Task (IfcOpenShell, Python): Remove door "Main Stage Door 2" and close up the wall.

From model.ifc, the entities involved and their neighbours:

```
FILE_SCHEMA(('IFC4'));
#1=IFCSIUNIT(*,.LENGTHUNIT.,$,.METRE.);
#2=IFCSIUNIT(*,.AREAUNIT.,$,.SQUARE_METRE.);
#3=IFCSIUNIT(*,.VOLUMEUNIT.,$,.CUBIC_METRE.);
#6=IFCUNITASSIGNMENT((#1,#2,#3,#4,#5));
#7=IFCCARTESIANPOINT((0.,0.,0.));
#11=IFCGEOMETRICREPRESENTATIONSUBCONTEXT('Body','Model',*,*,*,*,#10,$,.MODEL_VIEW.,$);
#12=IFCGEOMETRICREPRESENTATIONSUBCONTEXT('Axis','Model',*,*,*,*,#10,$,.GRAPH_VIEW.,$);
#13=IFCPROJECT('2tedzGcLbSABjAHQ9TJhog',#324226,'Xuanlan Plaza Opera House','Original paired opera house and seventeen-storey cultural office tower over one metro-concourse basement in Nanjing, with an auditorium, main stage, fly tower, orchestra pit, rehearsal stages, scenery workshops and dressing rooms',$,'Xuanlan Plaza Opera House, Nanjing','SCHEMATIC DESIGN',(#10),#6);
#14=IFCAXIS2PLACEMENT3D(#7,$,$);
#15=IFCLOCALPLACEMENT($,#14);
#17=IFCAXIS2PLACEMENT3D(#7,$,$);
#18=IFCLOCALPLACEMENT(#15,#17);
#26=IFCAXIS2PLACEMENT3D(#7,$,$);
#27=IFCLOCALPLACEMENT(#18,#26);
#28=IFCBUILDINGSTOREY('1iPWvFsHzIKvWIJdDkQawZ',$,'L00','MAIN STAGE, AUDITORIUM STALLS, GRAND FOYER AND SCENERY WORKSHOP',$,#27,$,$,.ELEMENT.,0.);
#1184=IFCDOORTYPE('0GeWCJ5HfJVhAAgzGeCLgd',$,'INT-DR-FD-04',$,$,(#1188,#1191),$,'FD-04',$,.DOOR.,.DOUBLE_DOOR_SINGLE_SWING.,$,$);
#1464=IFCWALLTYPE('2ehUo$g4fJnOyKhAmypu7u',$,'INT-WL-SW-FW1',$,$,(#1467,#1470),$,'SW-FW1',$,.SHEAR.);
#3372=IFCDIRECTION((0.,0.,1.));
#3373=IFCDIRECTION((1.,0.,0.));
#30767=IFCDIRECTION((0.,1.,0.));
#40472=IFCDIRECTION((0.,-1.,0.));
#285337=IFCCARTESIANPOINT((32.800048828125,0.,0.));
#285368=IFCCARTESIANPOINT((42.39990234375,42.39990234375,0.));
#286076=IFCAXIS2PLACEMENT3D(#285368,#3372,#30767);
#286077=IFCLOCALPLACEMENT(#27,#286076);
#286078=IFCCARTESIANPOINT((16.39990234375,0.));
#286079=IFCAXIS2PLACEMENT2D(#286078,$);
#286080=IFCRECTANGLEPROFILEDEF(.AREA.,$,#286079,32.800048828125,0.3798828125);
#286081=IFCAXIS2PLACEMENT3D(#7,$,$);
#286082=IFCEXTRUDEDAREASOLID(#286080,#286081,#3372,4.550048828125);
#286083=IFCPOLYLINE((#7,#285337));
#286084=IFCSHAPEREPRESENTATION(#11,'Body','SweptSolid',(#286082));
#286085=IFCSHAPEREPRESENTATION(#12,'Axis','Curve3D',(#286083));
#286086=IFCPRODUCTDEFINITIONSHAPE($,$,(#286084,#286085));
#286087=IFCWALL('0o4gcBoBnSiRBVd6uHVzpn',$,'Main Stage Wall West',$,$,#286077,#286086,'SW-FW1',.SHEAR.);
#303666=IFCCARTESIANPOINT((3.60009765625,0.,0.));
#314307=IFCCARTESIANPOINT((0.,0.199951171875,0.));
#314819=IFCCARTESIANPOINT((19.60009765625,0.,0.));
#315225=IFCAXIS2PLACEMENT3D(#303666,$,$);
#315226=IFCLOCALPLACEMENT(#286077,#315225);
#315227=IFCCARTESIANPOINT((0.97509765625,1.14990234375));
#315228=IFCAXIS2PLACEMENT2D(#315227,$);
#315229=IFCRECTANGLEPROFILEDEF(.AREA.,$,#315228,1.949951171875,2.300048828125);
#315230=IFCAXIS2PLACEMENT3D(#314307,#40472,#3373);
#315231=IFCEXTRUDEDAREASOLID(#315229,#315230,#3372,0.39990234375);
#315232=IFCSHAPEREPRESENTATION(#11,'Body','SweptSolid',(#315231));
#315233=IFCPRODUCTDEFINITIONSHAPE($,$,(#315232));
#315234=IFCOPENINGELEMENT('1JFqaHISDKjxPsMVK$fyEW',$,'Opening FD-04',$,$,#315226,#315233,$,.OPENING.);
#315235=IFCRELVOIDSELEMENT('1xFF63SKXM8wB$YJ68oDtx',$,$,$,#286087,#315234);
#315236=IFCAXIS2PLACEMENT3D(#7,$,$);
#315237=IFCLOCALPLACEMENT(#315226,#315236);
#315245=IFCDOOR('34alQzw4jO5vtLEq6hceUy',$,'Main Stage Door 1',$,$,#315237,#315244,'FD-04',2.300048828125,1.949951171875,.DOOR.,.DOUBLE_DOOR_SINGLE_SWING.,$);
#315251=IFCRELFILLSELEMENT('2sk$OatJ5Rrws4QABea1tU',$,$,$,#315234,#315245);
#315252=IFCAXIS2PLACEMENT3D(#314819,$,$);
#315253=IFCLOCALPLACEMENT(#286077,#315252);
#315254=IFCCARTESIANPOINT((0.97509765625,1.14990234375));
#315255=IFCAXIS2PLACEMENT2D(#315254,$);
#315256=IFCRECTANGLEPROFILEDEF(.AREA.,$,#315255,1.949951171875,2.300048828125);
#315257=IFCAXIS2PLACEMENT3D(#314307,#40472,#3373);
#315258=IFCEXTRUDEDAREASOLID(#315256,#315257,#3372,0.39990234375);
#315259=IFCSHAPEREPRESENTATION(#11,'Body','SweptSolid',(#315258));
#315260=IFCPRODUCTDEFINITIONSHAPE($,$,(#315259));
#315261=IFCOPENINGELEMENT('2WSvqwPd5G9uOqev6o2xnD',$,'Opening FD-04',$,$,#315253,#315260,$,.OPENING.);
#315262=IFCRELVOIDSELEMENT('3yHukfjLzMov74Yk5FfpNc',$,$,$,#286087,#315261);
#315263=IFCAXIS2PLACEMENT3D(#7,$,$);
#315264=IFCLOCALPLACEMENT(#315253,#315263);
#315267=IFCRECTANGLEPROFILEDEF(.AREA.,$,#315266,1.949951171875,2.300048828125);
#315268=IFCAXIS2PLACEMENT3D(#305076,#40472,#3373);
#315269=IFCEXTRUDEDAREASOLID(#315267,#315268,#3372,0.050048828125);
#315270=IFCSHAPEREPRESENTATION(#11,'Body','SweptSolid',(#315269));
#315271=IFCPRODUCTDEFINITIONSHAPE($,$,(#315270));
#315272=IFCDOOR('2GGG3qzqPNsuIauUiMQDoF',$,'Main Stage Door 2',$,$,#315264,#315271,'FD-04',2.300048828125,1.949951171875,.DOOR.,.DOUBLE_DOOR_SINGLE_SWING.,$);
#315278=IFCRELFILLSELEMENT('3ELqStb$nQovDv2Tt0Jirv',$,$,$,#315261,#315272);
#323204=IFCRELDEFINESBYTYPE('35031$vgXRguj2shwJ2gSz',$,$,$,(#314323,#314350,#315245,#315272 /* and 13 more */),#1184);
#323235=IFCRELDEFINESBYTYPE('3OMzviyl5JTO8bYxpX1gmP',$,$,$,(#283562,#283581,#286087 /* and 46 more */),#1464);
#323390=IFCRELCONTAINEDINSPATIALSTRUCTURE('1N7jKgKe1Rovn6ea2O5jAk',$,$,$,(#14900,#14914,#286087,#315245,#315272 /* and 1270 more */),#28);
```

```python
import ifcopenshell
import ifcopenshell.api.feature
import ifcopenshell.api.root
import ifcopenshell.geom
import ifcopenshell.util.shape

model = ifcopenshell.open("model.ifc")
settings = ifcopenshell.geom.settings()


def volume(element):
    """Net volume in cubic metres, openings subtracted."""
    shape = ifcopenshell.geom.create_shape(settings, element)
    return ifcopenshell.util.shape.get_volume(shape.geometry)


door = model.by_guid("2GGG3qzqPNsuIauUiMQDoF")
opening = door.FillsVoids[0].RelatingOpeningElement
wall = opening.VoidsElements[0].RelatingBuildingElement
before = volume(wall)

ifcopenshell.api.root.remove_product(model, product=door)
ifcopenshell.api.feature.remove_feature(model, feature=opening)

after = volume(wall)

print(f"wall volume {before:.3f} -> {after:.3f} m3")

model.write("model_rev.ifc")
```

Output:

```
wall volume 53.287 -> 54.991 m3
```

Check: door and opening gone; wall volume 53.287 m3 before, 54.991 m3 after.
